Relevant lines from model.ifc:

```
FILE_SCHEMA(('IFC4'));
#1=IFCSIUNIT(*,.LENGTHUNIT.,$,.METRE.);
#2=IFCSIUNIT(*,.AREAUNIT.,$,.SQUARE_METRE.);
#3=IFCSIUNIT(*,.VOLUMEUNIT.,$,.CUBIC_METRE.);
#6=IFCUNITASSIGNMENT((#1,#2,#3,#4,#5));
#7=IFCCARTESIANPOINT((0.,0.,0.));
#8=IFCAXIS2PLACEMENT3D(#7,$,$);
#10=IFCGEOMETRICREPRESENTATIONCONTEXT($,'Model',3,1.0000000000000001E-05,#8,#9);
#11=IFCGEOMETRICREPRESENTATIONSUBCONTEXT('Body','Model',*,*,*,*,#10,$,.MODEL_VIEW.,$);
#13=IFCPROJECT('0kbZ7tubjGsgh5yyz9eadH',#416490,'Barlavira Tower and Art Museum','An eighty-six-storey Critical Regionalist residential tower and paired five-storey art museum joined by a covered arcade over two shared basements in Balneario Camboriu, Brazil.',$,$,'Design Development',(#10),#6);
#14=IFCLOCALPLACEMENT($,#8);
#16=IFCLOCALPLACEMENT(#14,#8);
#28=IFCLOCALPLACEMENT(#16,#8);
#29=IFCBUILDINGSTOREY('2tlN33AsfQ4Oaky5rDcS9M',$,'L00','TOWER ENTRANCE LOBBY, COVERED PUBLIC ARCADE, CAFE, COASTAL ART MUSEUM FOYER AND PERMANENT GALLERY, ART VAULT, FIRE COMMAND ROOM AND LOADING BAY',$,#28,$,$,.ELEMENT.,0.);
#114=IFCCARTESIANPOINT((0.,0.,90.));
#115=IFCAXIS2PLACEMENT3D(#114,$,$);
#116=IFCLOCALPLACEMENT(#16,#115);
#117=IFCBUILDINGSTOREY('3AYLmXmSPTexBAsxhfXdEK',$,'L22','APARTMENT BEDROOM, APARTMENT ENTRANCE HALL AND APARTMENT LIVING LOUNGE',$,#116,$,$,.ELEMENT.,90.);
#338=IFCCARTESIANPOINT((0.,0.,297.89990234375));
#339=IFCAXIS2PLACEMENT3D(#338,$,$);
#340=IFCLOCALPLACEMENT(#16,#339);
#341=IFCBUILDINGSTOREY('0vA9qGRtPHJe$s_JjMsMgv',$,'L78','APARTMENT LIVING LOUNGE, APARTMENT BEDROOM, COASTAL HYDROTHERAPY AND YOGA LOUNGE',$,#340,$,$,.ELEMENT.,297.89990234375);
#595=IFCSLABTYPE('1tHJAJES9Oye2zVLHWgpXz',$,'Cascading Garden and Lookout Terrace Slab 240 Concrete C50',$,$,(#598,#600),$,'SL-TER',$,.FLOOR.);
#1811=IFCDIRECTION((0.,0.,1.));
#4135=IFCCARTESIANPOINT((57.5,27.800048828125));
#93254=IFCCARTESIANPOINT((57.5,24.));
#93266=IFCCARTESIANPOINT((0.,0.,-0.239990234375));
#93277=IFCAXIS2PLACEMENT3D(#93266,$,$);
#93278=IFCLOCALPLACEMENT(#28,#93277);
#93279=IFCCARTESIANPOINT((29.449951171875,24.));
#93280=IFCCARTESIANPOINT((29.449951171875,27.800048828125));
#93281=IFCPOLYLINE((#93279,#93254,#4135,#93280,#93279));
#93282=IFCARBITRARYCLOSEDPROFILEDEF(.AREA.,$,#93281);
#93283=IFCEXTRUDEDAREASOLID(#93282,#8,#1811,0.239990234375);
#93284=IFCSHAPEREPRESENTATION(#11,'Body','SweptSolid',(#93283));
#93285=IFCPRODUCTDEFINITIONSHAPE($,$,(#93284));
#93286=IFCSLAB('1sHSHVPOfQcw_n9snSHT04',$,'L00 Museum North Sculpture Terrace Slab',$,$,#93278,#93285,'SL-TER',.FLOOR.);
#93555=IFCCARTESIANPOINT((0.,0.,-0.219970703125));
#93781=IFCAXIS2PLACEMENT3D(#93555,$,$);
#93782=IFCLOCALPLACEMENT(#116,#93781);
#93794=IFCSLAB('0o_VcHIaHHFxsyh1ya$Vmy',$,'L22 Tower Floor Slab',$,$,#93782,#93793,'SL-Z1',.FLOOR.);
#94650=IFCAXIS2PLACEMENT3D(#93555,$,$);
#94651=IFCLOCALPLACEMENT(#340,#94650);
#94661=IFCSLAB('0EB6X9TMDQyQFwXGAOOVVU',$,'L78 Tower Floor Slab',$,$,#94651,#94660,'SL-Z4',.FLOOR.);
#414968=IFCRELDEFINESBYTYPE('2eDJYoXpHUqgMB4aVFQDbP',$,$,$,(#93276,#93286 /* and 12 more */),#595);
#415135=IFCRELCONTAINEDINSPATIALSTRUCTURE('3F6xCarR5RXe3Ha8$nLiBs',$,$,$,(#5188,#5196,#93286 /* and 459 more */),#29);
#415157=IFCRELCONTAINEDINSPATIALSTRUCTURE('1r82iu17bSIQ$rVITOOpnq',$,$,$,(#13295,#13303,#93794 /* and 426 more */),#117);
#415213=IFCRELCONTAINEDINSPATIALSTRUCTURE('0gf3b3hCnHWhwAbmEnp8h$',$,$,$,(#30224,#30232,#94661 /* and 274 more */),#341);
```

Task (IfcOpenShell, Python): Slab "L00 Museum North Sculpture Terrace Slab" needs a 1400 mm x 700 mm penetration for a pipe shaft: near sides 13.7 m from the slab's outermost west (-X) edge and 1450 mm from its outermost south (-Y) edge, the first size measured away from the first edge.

```python
import numpy as np
import ifcopenshell
import ifcopenshell.api.feature
import ifcopenshell.api.geometry
import ifcopenshell.api.root
import ifcopenshell.geom
import ifcopenshell.util.placement
import ifcopenshell.util.representation
import ifcopenshell.util.shape
import ifcopenshell.util.unit

model = ifcopenshell.open("model.ifc")
unit_scale = ifcopenshell.util.unit.calculate_unit_scale(model)
settings = ifcopenshell.geom.settings()


def volume(element):
    """Net volume in cubic metres, openings subtracted."""
    shape = ifcopenshell.geom.create_shape(settings, element)
    return ifcopenshell.util.shape.get_volume(shape.geometry)


slab = model.by_guid("1sHSHVPOfQcw_n9snSHT04")
before = volume(slab)

# Extent in the slab's own axes, in metres. The edges named are its -X and -Y sides.
slab_shape = ifcopenshell.geom.create_shape(settings, slab)
vertices = ifcopenshell.util.shape.get_vertices(slab_shape.geometry)
x_min, y_min, bottom = vertices.min(axis=0)
top = vertices[:, 2].max()

opening = ifcopenshell.api.root.create_entity(model, ifc_class="IfcOpeningElement", name="Pipe shaft opening", predefined_type="OPENING")
context = ifcopenshell.util.representation.get_context(model, "Model", "Body", "MODEL_VIEW")
width, depth = 1.4, 0.7
outline = [(0.0, 0.0), (width, 0.0), (width, depth), (0.0, depth), (0.0, 0.0)]
# Overshoot both faces by 50 mm so the cut is clean.
shape = ifcopenshell.api.geometry.add_slab_representation(
    model, context=context, depth=top - bottom + 0.1, polyline=outline
)
ifcopenshell.api.geometry.assign_representation(model, product=opening, representation=shape)

matrix = ifcopenshell.util.placement.get_local_placement(slab.ObjectPlacement)
matrix[:, 3] = matrix @ np.append(np.array([x_min + 13.7, y_min + 1.45, bottom - 0.05]) / unit_scale, 1.0)
ifcopenshell.api.geometry.edit_object_placement(model, product=opening, matrix=matrix, is_si=False)
ifcopenshell.api.feature.add_feature(model, feature=opening, element=slab)

after = volume(slab)

print(f"slab volume {before:.3f} -> {after:.3f} m3")

model.write("model_rev.ifc")
```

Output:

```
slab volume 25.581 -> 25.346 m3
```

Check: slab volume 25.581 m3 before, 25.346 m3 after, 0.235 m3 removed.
